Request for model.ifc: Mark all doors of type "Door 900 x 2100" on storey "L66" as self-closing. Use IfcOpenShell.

First a look at what the model holds.

```python
import ifcopenshell
import ifcopenshell.util.element

model = ifcopenshell.open("model.ifc")
print(model.schema)
storey = next(s for s in model.by_type("IfcBuildingStorey") if s.Name == "L66")
doors = [e for e in ifcopenshell.util.element.get_decomposition(storey) if e.is_a("IfcDoor")]
seen = {}
for e in doors:
    element_type = ifcopenshell.util.element.get_type(e)
    key = (element_type.Name if element_type != e and element_type else None, ifcopenshell.util.element.get_pset(e, "Pset_DoorCommon", "SelfClosing"))
    seen[key] = seen.get(key, 0) + 1
for (name, value), count in sorted(seen.items(), key=str):
    print(count, "x", name, "|", value)
```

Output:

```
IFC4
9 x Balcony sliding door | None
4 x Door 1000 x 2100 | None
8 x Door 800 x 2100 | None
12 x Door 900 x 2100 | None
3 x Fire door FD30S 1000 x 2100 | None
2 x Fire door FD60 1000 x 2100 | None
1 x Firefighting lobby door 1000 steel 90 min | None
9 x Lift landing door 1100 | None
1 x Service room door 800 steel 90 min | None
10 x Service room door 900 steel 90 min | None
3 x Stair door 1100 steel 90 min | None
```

```python
import ifcopenshell
import ifcopenshell.api.pset
import ifcopenshell.util.element

model = ifcopenshell.open("model.ifc")

storey = next(s for s in model.by_type("IfcBuildingStorey") if s.Name == "L66")
doors = [e for e in ifcopenshell.util.element.get_decomposition(storey) if e.is_a("IfcDoor")]

count = 0
for e in doors:
    element_type = ifcopenshell.util.element.get_type(e)
    if element_type in (None, e) or element_type.Name != "Door 900 x 2100":
        continue
    found = ifcopenshell.util.element.get_pset(e, "Pset_DoorCommon", should_inherit=False)
    if found:
        pset = model.by_id(found["id"])
        if len(ifcopenshell.util.element.get_elements_by_pset(pset)) > 1:
            pset = ifcopenshell.api.pset.unshare_pset(model, products=[e], pset=pset)[0]
    else:
        pset = ifcopenshell.api.pset.add_pset(model, product=e, name="Pset_DoorCommon")
    ifcopenshell.api.pset.edit_pset(model, pset=pset, properties={"SelfClosing": True})
    count += 1

print(count, "doors updated")

model.write("model-out.ifc")
```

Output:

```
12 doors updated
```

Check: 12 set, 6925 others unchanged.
